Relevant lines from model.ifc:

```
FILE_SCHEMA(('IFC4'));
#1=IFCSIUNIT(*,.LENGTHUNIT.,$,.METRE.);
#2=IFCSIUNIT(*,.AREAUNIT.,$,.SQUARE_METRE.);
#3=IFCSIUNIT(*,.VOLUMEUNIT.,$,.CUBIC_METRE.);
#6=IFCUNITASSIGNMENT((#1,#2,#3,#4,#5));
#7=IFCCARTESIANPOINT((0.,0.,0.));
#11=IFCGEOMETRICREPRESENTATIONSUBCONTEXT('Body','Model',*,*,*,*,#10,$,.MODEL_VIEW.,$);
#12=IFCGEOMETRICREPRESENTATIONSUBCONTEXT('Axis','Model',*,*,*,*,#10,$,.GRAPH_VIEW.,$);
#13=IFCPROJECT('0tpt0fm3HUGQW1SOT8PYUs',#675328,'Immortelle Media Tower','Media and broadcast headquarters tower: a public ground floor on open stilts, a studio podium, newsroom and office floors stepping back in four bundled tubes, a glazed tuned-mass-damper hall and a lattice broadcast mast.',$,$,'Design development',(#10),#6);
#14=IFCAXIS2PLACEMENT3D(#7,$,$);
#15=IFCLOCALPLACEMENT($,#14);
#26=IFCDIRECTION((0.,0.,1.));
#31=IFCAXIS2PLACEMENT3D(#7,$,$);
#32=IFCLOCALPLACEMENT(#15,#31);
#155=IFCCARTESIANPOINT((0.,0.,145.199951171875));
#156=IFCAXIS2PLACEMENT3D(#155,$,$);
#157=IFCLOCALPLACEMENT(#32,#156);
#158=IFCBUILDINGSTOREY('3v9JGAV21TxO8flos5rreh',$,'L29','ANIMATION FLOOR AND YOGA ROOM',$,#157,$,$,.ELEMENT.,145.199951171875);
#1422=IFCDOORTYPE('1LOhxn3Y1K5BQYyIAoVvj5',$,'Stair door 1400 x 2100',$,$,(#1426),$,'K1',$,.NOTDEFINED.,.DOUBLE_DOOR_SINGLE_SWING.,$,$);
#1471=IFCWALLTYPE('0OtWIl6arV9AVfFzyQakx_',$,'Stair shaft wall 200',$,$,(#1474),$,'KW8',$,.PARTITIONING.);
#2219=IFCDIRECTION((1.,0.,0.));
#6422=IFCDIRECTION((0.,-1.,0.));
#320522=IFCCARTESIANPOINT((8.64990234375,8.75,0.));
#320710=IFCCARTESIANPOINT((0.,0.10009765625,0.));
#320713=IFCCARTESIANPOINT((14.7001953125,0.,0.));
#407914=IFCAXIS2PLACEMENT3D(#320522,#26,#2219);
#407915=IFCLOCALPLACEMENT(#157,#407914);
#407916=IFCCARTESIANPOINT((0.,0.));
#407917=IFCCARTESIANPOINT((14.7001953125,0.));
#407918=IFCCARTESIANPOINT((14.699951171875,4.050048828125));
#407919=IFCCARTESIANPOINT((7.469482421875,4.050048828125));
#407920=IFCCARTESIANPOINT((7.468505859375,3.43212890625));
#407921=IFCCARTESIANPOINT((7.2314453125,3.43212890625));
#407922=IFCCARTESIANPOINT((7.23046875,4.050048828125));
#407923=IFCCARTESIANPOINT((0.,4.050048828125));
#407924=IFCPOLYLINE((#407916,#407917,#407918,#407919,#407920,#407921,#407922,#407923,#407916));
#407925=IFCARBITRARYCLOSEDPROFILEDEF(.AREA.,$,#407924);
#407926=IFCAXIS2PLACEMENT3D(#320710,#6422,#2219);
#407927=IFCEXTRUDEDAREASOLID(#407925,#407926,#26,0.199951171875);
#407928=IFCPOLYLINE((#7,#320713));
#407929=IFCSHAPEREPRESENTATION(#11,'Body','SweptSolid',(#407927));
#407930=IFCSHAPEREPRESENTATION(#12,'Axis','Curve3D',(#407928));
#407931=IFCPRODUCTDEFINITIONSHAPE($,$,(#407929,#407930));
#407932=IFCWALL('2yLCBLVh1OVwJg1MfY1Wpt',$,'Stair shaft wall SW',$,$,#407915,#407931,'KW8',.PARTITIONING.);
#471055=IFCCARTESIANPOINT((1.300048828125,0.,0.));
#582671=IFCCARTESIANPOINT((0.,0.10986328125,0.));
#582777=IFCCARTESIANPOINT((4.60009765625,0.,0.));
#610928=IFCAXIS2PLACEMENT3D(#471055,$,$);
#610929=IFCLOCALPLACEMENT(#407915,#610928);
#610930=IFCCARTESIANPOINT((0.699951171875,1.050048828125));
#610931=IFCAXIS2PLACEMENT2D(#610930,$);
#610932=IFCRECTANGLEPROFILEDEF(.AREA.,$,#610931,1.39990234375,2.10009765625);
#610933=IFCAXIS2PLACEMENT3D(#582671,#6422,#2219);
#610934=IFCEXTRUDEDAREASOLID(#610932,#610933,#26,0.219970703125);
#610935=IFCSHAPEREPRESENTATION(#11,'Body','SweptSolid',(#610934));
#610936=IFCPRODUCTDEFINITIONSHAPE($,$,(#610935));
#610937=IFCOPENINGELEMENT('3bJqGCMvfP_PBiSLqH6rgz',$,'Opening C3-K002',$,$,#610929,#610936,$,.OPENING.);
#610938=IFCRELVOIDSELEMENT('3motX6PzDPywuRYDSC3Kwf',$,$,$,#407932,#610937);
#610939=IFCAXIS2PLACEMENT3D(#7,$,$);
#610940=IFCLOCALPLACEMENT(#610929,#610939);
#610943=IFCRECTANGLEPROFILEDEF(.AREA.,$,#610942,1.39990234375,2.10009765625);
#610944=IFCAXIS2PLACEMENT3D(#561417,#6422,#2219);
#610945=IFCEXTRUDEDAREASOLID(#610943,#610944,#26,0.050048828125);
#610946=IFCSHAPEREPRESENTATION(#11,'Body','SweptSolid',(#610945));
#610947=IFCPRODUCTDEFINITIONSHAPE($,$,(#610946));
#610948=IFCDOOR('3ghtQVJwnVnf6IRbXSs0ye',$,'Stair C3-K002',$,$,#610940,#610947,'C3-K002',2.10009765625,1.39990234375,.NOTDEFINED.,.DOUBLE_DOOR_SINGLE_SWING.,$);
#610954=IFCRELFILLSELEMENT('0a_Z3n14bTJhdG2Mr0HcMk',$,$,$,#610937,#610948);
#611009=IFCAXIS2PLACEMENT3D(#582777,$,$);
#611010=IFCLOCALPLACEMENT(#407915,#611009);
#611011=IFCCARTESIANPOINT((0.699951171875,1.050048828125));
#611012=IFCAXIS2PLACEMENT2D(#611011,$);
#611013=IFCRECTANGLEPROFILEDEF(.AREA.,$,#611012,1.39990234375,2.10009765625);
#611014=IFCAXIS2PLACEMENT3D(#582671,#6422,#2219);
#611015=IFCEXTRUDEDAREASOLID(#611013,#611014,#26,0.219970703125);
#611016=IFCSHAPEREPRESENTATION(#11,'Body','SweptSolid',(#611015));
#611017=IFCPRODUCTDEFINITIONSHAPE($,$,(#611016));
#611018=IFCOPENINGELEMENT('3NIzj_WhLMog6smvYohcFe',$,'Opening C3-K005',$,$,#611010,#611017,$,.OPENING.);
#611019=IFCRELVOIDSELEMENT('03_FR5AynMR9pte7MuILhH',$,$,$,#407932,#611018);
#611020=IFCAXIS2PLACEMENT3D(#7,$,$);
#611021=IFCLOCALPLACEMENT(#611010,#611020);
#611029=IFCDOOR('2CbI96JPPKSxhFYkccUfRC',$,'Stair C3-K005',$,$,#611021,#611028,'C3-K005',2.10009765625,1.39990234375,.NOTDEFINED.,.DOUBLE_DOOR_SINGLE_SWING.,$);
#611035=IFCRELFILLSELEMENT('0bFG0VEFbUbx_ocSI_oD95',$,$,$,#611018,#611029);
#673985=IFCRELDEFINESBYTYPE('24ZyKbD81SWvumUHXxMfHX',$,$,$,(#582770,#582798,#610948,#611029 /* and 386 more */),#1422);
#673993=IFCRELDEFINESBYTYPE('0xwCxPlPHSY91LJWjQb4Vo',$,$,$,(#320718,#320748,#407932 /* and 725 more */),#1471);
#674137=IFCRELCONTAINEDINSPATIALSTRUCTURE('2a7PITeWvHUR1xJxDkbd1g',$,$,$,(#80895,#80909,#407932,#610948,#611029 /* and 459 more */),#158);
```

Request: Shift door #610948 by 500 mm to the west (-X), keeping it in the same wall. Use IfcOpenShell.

```python
import ifcopenshell
import ifcopenshell.api.geometry
import ifcopenshell.util.placement

model = ifcopenshell.open("model.ifc")

door = model.by_guid("3ghtQVJwnVnf6IRbXSs0ye")
opening = door.FillsVoids[0].RelatingOpeningElement
wall = opening.VoidsElements[0].RelatingBuildingElement

wall_matrix = ifcopenshell.util.placement.get_local_placement(wall.ObjectPlacement)
shift = wall_matrix[:3, 0] * -0.5
before = ifcopenshell.util.placement.get_local_placement(door.ObjectPlacement)[:3, 3].copy()

# The door is placed relative to its opening, so it follows when the opening moves.
matrix = ifcopenshell.util.placement.get_local_placement(opening.ObjectPlacement)
matrix[:3, 3] += shift
ifcopenshell.api.geometry.edit_object_placement(
    model, product=opening, matrix=matrix, is_si=False, should_transform_children=True
)

after = ifcopenshell.util.placement.get_local_placement(door.ObjectPlacement)[:3, 3]
print("door moved by", (after - before).round(3) + 0.0)

model.write("model_v2.ifc")
```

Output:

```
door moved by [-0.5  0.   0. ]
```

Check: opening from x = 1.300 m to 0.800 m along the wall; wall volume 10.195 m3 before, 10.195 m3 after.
